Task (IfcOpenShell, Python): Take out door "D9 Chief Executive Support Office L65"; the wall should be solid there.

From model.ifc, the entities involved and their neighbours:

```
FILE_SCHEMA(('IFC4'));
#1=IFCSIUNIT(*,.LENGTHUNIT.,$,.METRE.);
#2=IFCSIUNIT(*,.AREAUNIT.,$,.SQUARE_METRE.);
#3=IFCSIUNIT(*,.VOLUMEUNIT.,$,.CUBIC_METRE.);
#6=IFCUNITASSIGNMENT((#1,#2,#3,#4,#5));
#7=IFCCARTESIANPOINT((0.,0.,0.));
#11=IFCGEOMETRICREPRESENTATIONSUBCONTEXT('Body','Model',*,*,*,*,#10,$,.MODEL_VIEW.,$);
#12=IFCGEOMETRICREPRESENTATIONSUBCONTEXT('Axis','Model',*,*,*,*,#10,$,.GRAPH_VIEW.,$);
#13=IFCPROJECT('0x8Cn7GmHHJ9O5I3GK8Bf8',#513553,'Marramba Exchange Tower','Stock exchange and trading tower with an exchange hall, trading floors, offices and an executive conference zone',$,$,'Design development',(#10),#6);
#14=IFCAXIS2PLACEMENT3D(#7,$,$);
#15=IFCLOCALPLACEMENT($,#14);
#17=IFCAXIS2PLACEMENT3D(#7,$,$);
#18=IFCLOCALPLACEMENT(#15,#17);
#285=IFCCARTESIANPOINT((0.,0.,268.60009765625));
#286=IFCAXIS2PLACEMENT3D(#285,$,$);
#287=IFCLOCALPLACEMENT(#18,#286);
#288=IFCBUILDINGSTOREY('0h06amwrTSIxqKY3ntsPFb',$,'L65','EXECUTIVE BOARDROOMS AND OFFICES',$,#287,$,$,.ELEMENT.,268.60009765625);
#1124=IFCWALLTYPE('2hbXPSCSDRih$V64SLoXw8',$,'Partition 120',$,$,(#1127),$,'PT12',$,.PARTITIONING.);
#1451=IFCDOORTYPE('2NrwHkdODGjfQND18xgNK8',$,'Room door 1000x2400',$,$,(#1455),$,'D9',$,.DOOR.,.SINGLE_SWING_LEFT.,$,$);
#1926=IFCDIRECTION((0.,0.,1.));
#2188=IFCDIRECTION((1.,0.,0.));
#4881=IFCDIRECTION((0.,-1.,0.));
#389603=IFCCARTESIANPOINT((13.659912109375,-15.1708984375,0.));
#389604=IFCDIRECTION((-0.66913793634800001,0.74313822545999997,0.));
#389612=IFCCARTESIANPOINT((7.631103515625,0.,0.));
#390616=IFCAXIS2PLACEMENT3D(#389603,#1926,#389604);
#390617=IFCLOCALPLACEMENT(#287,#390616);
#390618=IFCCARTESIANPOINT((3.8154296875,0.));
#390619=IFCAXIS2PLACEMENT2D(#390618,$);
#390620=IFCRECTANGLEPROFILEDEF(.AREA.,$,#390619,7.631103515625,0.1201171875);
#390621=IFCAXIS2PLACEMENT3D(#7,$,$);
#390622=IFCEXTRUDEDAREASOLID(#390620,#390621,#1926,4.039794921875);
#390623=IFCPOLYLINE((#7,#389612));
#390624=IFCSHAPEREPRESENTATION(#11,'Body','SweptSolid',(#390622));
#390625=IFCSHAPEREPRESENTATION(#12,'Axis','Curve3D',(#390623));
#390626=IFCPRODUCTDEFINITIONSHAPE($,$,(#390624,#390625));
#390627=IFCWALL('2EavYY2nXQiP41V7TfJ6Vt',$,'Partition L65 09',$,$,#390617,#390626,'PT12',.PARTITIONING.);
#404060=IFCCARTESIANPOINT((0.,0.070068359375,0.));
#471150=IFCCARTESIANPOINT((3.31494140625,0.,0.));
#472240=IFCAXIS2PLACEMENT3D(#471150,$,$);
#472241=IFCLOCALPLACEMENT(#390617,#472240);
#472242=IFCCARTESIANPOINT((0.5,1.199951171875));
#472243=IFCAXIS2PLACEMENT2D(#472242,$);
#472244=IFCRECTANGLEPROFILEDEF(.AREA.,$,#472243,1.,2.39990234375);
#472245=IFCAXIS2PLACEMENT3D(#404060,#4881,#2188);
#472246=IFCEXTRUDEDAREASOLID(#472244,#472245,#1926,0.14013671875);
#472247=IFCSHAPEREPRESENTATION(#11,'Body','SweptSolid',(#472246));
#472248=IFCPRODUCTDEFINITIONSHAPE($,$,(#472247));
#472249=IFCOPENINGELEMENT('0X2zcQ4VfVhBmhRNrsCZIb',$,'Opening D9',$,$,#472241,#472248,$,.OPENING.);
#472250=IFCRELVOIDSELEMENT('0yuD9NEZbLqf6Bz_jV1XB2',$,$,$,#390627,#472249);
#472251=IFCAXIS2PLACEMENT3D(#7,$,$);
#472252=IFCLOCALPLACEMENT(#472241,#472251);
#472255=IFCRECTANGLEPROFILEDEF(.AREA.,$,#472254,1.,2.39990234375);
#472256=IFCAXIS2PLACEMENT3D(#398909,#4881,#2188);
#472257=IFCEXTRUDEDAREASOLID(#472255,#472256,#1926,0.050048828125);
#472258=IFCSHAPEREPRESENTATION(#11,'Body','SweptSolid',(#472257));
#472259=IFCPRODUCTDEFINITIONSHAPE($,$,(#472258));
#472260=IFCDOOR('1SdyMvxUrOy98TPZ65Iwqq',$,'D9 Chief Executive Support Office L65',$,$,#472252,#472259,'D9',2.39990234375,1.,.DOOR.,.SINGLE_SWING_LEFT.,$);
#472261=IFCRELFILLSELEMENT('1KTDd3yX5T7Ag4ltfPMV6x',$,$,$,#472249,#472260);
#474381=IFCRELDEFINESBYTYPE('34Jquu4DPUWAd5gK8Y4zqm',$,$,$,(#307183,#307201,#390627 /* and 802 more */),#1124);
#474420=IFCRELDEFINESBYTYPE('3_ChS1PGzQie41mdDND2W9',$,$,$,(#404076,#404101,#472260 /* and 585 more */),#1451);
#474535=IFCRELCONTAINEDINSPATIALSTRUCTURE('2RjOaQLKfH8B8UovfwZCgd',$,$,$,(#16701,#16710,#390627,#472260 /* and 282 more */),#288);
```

```python
import ifcopenshell
import ifcopenshell.api.feature
import ifcopenshell.api.root
import ifcopenshell.geom
import ifcopenshell.util.shape

model = ifcopenshell.open("model.ifc")
settings = ifcopenshell.geom.settings()


def volume(element):
    """Net volume in cubic metres, openings subtracted."""
    shape = ifcopenshell.geom.create_shape(settings, element)
    return ifcopenshell.util.shape.get_volume(shape.geometry)


door = model.by_guid("1SdyMvxUrOy98TPZ65Iwqq")
opening = door.FillsVoids[0].RelatingOpeningElement
wall = opening.VoidsElements[0].RelatingBuildingElement
before = volume(wall)

ifcopenshell.api.root.remove_product(model, product=door)
ifcopenshell.api.feature.remove_feature(model, feature=opening)

after = volume(wall)

print(f"wall volume {before:.3f} -> {after:.3f} m3")

model.write("model_edited.ifc")
```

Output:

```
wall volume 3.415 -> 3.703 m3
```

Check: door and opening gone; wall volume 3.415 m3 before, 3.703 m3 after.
